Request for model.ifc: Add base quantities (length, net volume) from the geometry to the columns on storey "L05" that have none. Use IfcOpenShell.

First a look at what the model holds.

```python
import ifcopenshell
import ifcopenshell.util.element
import ifcopenshell.util.unit

model = ifcopenshell.open("model.ifc")
print(model.schema)
for unit_type in ("LENGTHUNIT", "AREAUNIT", "VOLUMEUNIT"):
    print(unit_type, ifcopenshell.util.unit.calculate_unit_scale(model, unit_type))
storey = next(s for s in model.by_type("IfcBuildingStorey") if s.Name == "L05")
columns = [e for e in ifcopenshell.util.element.get_decomposition(storey) if e.is_a("IfcColumn")]
for e in sorted(columns, key=lambda e: e.id()):
    print(e.id(), e.is_a(), e.Name, list(ifcopenshell.util.element.get_psets(e, qtos_only=True)), sep=" | ")
```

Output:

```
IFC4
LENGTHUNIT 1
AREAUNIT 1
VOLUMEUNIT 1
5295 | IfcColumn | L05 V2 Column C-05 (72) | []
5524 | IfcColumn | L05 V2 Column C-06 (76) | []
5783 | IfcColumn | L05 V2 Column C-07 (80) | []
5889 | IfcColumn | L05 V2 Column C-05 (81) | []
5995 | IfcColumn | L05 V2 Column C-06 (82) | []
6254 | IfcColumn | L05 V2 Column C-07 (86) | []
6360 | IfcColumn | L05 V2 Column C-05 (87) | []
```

```python
import ifcopenshell
import ifcopenshell.api.pset
import ifcopenshell.geom
import ifcopenshell.util.element
import ifcopenshell.util.shape
import ifcopenshell.util.unit

model = ifcopenshell.open("model.ifc")
unit_scale = ifcopenshell.util.unit.calculate_unit_scale(model)
volume_scale = ifcopenshell.util.unit.calculate_unit_scale(model, "VOLUMEUNIT")
settings = ifcopenshell.geom.settings()

storey = next(s for s in model.by_type("IfcBuildingStorey") if s.Name == "L05")
columns = [e for e in ifcopenshell.util.element.get_decomposition(storey) if e.is_a("IfcColumn")]

for e in sorted(columns, key=lambda e: e.id()):
    if ifcopenshell.util.element.get_psets(e, qtos_only=True, should_inherit=False):
        continue
    # Geometry comes back in metres, in the element's own axes.
    shape = ifcopenshell.geom.create_shape(settings, e)
    values = {
        "Length": ifcopenshell.util.shape.get_z(shape.geometry) / unit_scale,
        "NetVolume": ifcopenshell.util.shape.get_volume(shape.geometry) / volume_scale,
    }
    qto = ifcopenshell.api.pset.add_qto(model, product=e, name="Qto_ColumnBaseQuantities")
    ifcopenshell.api.pset.edit_qto(model, qto=qto, properties=values)
    print(e.id(), {k: round(v, 3) for k, v in values.items()})

model.write("model_edited.ifc")
```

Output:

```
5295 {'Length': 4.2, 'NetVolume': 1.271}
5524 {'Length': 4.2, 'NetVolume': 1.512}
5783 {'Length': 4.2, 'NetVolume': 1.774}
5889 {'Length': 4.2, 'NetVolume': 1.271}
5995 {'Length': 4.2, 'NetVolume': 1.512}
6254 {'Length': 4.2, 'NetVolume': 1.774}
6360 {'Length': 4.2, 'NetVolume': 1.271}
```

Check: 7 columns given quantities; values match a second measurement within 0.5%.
